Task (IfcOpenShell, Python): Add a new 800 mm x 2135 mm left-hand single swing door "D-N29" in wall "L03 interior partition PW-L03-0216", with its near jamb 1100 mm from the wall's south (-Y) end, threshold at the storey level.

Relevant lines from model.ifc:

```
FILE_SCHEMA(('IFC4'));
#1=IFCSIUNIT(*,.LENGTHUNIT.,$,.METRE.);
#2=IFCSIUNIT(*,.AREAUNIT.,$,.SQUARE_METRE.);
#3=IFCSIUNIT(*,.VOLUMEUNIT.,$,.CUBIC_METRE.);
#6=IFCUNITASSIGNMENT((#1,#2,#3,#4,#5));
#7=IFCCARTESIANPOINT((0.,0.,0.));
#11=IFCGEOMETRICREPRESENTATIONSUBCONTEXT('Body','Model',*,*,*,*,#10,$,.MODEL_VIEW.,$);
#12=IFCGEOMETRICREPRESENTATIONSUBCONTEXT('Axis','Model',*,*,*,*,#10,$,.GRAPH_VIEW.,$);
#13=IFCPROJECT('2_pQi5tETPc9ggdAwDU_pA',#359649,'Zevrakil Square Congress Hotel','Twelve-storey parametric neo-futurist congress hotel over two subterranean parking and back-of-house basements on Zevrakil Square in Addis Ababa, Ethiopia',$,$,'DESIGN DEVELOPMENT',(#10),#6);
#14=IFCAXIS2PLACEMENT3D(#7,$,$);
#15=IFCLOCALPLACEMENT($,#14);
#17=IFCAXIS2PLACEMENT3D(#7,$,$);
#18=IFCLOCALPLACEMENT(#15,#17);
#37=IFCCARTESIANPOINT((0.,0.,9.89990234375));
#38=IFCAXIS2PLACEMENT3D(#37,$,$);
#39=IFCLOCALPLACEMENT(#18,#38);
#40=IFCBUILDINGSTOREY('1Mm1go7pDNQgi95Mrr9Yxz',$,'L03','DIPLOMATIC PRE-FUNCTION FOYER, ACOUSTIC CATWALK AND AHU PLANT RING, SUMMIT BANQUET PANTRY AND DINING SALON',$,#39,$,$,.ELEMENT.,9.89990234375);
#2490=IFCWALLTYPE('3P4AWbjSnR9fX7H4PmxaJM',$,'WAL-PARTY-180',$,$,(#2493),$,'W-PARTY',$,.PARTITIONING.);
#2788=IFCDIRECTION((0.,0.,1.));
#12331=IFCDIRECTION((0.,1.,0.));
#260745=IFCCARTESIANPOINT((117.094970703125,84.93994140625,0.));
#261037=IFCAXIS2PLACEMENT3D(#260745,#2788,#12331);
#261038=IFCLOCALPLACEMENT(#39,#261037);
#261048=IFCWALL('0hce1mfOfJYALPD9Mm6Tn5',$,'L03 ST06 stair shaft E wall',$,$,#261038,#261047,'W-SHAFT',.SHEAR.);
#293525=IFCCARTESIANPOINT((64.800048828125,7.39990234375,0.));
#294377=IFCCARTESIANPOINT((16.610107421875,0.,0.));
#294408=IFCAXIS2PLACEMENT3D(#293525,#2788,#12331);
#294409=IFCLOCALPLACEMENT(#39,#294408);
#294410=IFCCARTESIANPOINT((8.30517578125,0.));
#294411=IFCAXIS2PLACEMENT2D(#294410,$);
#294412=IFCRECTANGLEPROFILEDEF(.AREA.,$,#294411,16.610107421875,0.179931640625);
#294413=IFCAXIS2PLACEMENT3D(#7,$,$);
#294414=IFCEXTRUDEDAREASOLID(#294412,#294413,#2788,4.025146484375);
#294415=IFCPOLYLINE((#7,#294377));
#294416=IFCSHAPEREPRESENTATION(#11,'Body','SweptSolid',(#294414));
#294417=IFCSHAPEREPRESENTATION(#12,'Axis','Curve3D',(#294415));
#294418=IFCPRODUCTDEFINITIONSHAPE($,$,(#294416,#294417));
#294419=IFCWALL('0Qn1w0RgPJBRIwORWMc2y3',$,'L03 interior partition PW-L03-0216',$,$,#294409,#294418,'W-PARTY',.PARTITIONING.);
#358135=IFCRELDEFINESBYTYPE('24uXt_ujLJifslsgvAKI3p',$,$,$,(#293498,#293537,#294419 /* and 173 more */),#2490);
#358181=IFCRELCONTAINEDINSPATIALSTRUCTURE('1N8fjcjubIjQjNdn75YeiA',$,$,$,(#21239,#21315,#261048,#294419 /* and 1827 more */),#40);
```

```python
import numpy as np
import ifcopenshell
import ifcopenshell.api.feature
import ifcopenshell.api.geometry
import ifcopenshell.api.root
import ifcopenshell.api.spatial
import ifcopenshell.geom
import ifcopenshell.util.element
import ifcopenshell.util.placement
import ifcopenshell.util.representation
import ifcopenshell.util.shape
import ifcopenshell.util.unit

model = ifcopenshell.open("model.ifc")
unit_scale = ifcopenshell.util.unit.calculate_unit_scale(model)
settings = ifcopenshell.geom.settings()


def volume(element):
    """Net volume in cubic metres, openings subtracted."""
    shape = ifcopenshell.geom.create_shape(settings, element)
    return ifcopenshell.util.shape.get_volume(shape.geometry)


wall = model.by_guid("0Qn1w0RgPJBRIwORWMc2y3")
storey = ifcopenshell.util.element.get_container(wall, ifc_class="IfcBuildingStorey")
context = ifcopenshell.util.representation.get_context(model, "Model", "Body", "MODEL_VIEW")
before = volume(wall)

width, height, from_end, sill = 0.8, 2.135, 1.1, 0.0  # metres

# The wall runs along its own X axis, and the end named is its -X end.
wall_shape = ifcopenshell.geom.create_shape(settings, wall)
x, y, z = ifcopenshell.util.shape.get_vertices(wall_shape.geometry).T
start = x.min() + from_end
face, thickness = float(y.min()), float(y.max() - y.min())
wall_matrix = ifcopenshell.util.placement.get_local_placement(wall.ObjectPlacement)
level = ifcopenshell.util.placement.get_local_placement(storey.ObjectPlacement)[2, 3]


def in_wall(x, y):
    """Placement at x, y metres in the wall's axes, at sill height."""
    matrix = wall_matrix.copy()
    matrix[:, 3] = wall_matrix @ np.array([x / unit_scale, y / unit_scale, 0.0, 1.0])
    matrix[2, 3] = level + sill / unit_scale
    return matrix


# Opening: a box that overshoots both wall faces by 50 mm.
opening = ifcopenshell.api.root.create_entity(model, ifc_class="IfcOpeningElement", predefined_type="OPENING")
box = ifcopenshell.api.geometry.add_wall_representation(
    model, context=context, length=width, height=height, thickness=thickness + 0.1
)
ifcopenshell.api.geometry.assign_representation(model, product=opening, representation=box)
ifcopenshell.api.geometry.edit_object_placement(model, product=opening, matrix=in_wall(start, face - 0.05), is_si=False)
ifcopenshell.api.feature.add_feature(model, feature=opening, element=wall)

door = ifcopenshell.api.root.create_entity(model, ifc_class="IfcDoor", name="D-N29", predefined_type="DOOR")
door.OverallWidth, door.OverallHeight = width / unit_scale, height / unit_scale
door.OperationType = "SINGLE_SWING_LEFT"
body = ifcopenshell.api.geometry.add_door_representation(
    model,
    context=context,
    overall_width=door.OverallWidth,
    overall_height=door.OverallHeight,
    operation_type="SINGLE_SWING_LEFT",
    lining_properties={"LiningDepth": thickness / unit_scale, "ThresholdDepth": thickness / unit_scale},
)
ifcopenshell.api.geometry.assign_representation(model, product=door, representation=body)
ifcopenshell.api.spatial.assign_container(model, products=[door], relating_structure=storey)
ifcopenshell.api.feature.add_filling(model, opening=opening, element=door)

# The lining spans the wall, so the door starts at the wall face.
ifcopenshell.api.geometry.edit_object_placement(model, product=door, matrix=in_wall(start, face), is_si=False)

after = volume(wall)

print(f"wall volume {before:.3f} -> {after:.3f} m3")

model.write("model-out.ifc")
```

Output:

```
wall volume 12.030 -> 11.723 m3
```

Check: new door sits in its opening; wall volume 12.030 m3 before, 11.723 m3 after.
